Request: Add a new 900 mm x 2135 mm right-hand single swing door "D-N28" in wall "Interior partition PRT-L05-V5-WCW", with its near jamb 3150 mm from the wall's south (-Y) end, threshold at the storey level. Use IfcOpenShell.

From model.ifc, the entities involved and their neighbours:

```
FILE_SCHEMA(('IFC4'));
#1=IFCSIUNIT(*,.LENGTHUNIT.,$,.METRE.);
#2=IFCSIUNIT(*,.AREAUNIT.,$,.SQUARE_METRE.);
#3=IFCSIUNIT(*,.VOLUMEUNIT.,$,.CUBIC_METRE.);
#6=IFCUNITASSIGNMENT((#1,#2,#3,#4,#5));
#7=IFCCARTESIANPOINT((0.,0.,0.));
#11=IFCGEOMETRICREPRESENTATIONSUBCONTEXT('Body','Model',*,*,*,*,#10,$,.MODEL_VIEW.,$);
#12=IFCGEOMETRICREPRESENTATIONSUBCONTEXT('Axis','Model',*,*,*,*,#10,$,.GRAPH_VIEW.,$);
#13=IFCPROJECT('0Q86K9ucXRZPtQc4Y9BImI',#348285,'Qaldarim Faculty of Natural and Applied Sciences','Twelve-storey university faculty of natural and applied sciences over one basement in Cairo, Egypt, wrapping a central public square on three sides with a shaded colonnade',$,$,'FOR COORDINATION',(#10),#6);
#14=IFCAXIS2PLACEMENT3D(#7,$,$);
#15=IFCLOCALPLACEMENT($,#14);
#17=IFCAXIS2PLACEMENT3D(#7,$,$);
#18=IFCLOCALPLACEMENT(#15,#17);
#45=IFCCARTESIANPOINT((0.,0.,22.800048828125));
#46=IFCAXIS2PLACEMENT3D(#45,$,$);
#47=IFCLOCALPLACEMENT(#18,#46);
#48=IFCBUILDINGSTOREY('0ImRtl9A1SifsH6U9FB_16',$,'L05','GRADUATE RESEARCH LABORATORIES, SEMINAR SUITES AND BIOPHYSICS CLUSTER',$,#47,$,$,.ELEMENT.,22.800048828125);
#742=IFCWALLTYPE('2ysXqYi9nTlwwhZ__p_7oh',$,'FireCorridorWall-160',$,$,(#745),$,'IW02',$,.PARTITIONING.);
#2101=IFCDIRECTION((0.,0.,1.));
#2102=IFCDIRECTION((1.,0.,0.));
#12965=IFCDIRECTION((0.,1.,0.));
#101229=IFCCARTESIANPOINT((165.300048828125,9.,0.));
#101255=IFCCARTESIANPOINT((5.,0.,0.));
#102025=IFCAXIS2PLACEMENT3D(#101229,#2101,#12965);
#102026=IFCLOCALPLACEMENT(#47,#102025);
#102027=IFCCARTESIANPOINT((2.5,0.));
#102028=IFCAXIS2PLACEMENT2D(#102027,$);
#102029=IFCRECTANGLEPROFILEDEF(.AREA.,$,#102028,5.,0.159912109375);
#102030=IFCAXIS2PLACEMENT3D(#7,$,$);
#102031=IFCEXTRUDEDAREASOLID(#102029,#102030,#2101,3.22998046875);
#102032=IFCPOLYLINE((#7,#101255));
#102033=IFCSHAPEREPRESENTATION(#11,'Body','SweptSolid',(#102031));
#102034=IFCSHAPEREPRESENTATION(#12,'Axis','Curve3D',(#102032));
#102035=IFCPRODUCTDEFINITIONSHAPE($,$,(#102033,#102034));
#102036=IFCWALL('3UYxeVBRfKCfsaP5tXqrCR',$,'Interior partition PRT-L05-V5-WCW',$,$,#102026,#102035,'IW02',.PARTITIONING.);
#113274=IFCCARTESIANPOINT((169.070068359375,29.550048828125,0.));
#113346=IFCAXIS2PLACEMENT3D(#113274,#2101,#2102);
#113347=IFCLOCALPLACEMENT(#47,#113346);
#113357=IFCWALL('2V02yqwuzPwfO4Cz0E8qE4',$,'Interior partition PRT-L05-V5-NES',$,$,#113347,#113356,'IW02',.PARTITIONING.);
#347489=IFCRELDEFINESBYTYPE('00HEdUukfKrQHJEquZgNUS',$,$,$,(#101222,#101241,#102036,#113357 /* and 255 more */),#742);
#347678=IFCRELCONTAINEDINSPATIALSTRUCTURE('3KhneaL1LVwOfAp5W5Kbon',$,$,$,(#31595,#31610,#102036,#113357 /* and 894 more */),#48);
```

```python
import numpy as np
import ifcopenshell
import ifcopenshell.api.feature
import ifcopenshell.api.geometry
import ifcopenshell.api.root
import ifcopenshell.api.spatial
import ifcopenshell.geom
import ifcopenshell.util.element
import ifcopenshell.util.placement
import ifcopenshell.util.representation
import ifcopenshell.util.shape
import ifcopenshell.util.unit

model = ifcopenshell.open("model.ifc")
unit_scale = ifcopenshell.util.unit.calculate_unit_scale(model)
settings = ifcopenshell.geom.settings()


def volume(element):
    """Net volume in cubic metres, openings subtracted."""
    shape = ifcopenshell.geom.create_shape(settings, element)
    return ifcopenshell.util.shape.get_volume(shape.geometry)


wall = model.by_id(102036)
storey = ifcopenshell.util.element.get_container(wall, ifc_class="IfcBuildingStorey")
context = ifcopenshell.util.representation.get_context(model, "Model", "Body", "MODEL_VIEW")
before = volume(wall)

width, height, from_end, sill = 0.9, 2.135, 3.15, 0.0  # metres

# The wall runs along its own X axis, and the end named is its -X end.
wall_shape = ifcopenshell.geom.create_shape(settings, wall)
x, y, z = ifcopenshell.util.shape.get_vertices(wall_shape.geometry).T
start = x.min() + from_end
face, thickness = float(y.min()), float(y.max() - y.min())
wall_matrix = ifcopenshell.util.placement.get_local_placement(wall.ObjectPlacement)
level = ifcopenshell.util.placement.get_local_placement(storey.ObjectPlacement)[2, 3]


def in_wall(x, y):
    """Placement at x, y metres in the wall's axes, at sill height."""
    matrix = wall_matrix.copy()
    matrix[:, 3] = wall_matrix @ np.array([x / unit_scale, y / unit_scale, 0.0, 1.0])
    matrix[2, 3] = level + sill / unit_scale
    return matrix


# Opening: a box that overshoots both wall faces by 50 mm.
opening = ifcopenshell.api.root.create_entity(model, ifc_class="IfcOpeningElement", predefined_type="OPENING")
box = ifcopenshell.api.geometry.add_wall_representation(
    model, context=context, length=width, height=height, thickness=thickness + 0.1
)
ifcopenshell.api.geometry.assign_representation(model, product=opening, representation=box)
ifcopenshell.api.geometry.edit_object_placement(model, product=opening, matrix=in_wall(start, face - 0.05), is_si=False)
ifcopenshell.api.feature.add_feature(model, feature=opening, element=wall)

door = ifcopenshell.api.root.create_entity(model, ifc_class="IfcDoor", name="D-N28", predefined_type="DOOR")
door.OverallWidth, door.OverallHeight = width / unit_scale, height / unit_scale
door.OperationType = "SINGLE_SWING_RIGHT"
body = ifcopenshell.api.geometry.add_door_representation(
    model,
    context=context,
    overall_width=door.OverallWidth,
    overall_height=door.OverallHeight,
    operation_type="SINGLE_SWING_RIGHT",
    lining_properties={"LiningDepth": thickness / unit_scale, "ThresholdDepth": thickness / unit_scale},
)
ifcopenshell.api.geometry.assign_representation(model, product=door, representation=body)
ifcopenshell.api.spatial.assign_container(model, products=[door], relating_structure=storey)
ifcopenshell.api.feature.add_filling(model, opening=opening, element=door)

# The lining spans the wall, so the door starts at the wall face.
ifcopenshell.api.geometry.edit_object_placement(model, product=door, matrix=in_wall(start, face), is_si=False)

after = volume(wall)

print(f"wall volume {before:.3f} -> {after:.3f} m3")

model.write("model_edited.ifc")
```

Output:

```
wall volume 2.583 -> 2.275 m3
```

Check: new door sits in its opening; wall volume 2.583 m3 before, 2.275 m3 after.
